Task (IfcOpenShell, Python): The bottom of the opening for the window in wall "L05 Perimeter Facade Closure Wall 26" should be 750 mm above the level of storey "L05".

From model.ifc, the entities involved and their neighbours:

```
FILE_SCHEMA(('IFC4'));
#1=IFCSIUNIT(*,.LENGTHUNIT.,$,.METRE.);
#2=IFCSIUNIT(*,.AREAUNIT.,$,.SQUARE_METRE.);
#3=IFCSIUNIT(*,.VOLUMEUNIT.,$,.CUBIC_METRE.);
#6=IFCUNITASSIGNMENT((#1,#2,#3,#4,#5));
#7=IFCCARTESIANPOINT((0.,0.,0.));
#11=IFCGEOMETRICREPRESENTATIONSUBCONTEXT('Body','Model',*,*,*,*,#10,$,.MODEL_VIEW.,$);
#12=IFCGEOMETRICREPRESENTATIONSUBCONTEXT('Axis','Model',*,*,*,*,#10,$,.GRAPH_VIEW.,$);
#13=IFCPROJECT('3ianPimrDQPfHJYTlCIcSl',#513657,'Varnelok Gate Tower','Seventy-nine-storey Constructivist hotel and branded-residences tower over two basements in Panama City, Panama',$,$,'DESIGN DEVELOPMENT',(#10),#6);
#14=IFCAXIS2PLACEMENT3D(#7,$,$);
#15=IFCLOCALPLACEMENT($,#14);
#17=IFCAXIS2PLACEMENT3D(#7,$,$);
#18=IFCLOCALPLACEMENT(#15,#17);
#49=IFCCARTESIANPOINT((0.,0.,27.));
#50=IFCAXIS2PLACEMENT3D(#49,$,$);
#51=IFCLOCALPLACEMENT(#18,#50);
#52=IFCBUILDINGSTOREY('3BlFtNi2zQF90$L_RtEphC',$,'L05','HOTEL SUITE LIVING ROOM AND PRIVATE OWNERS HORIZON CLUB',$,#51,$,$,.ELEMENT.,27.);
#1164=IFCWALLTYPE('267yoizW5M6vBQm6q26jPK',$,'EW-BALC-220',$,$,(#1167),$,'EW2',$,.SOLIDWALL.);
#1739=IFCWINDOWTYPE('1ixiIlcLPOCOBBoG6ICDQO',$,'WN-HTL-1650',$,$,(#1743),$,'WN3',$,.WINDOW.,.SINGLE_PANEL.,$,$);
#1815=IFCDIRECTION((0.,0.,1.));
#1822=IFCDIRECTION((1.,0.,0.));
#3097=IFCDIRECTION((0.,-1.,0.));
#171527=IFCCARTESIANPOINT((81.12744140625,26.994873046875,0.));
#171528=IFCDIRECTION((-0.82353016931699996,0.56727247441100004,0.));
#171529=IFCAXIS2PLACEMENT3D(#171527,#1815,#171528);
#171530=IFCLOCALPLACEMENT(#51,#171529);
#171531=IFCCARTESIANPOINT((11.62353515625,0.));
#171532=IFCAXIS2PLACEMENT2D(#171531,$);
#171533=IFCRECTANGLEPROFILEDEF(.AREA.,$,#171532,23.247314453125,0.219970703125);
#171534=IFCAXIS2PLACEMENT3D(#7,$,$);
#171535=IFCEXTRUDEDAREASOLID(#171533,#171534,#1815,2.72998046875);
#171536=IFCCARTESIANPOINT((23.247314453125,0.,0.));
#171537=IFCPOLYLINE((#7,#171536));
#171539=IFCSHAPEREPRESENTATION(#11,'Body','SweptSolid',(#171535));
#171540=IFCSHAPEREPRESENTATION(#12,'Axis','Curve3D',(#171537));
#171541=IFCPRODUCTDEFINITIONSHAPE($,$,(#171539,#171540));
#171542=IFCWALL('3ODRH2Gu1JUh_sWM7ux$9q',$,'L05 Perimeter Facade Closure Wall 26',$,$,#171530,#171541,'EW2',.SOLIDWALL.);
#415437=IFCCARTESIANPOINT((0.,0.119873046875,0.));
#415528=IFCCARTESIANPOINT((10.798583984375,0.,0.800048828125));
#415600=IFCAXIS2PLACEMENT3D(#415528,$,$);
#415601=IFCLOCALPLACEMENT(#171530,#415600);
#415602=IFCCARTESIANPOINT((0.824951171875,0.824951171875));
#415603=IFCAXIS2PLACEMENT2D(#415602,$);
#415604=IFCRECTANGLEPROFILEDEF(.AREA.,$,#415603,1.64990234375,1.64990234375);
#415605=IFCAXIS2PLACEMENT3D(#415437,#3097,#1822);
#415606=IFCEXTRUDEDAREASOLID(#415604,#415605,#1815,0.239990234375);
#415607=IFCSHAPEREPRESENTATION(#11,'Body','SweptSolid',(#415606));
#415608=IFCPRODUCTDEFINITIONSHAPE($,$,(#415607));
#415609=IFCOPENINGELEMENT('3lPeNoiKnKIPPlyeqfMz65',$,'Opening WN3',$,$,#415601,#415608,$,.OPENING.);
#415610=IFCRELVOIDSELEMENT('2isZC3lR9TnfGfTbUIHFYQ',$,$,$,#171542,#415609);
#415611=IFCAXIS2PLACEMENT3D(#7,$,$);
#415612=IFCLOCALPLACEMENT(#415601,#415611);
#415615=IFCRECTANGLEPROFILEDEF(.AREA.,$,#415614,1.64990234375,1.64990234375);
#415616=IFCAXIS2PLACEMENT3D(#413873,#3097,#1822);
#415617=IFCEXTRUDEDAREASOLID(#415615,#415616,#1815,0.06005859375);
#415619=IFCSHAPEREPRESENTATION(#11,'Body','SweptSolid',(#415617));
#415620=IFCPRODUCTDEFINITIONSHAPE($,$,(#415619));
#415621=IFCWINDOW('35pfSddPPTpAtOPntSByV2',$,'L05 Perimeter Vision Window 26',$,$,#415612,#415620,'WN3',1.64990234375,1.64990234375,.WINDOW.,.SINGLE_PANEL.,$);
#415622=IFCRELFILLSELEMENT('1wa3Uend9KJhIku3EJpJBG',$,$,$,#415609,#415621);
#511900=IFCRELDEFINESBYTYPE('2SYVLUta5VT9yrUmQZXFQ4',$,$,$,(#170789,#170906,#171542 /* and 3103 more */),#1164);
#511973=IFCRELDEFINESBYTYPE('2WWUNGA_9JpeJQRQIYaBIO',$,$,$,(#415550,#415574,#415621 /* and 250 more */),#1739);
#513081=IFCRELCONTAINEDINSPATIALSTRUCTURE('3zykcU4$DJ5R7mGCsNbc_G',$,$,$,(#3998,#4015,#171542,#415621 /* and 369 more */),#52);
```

```python
import numpy as np
import ifcopenshell
import ifcopenshell.api.geometry
import ifcopenshell.geom
import ifcopenshell.util.element
import ifcopenshell.util.placement
import ifcopenshell.util.shape
import ifcopenshell.util.unit

model = ifcopenshell.open("model.ifc")
unit_scale = ifcopenshell.util.unit.calculate_unit_scale(model)

window = model.by_guid("35pfSddPPTpAtOPntSByV2")
opening = window.FillsVoids[0].RelatingOpeningElement
storey = ifcopenshell.util.element.get_container(window, ifc_class="IfcBuildingStorey")
level = ifcopenshell.util.placement.get_local_placement(storey.ObjectPlacement)[2, 3]

# The opening's origin need not be at the sill, so measure its lowest point.
shape = ifcopenshell.geom.create_shape(ifcopenshell.geom.settings(), opening)
bottom = ifcopenshell.util.shape.get_shape_bottom_elevation(shape, shape.geometry) / unit_scale
dz = level + 0.75 - bottom

shift = np.array([0.0, 0.0, dz])
# The window is placed relative to its opening, so it follows when the opening moves.
matrix = ifcopenshell.util.placement.get_local_placement(opening.ObjectPlacement)
matrix[:3, 3] += shift
ifcopenshell.api.geometry.edit_object_placement(
    model, product=opening, matrix=matrix, is_si=False, should_transform_children=True
)

print(f"moved by {dz * unit_scale:+.3f} m")

model.write("model-out.ifc")
```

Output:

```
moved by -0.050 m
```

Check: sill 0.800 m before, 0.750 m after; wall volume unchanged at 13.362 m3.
